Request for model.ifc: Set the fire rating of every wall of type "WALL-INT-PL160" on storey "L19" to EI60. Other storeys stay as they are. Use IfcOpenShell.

First a look at what the model holds.

```python
import ifcopenshell
import ifcopenshell.util.element

model = ifcopenshell.open("model.ifc")
print(model.schema)
storey = next(s for s in model.by_type("IfcBuildingStorey") if s.Name == "L19")
walls = [e for e in ifcopenshell.util.element.get_decomposition(storey) if e.is_a("IfcWall")]
seen = {}
for e in walls:
    element_type = ifcopenshell.util.element.get_type(e)
    key = (element_type.Name if element_type != e and element_type else None, ifcopenshell.util.element.get_pset(e, "Pset_WallCommon", "FireRating"))
    seen[key] = seen.get(key, 0) + 1
for (name, value), count in sorted(seen.items(), key=str):
    print(count, "x", name, "|", value)
```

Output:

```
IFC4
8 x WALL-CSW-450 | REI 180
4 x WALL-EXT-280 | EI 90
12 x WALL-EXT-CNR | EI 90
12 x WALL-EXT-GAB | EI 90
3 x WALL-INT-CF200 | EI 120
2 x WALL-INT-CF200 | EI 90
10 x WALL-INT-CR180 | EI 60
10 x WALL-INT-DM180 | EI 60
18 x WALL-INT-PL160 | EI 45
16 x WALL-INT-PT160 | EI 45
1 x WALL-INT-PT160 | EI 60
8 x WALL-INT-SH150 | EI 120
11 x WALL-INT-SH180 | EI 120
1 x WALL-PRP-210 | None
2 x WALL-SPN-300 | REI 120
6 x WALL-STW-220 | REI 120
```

```python
import ifcopenshell
import ifcopenshell.api.pset
import ifcopenshell.util.element

model = ifcopenshell.open("model.ifc")

storey = next(s for s in model.by_type("IfcBuildingStorey") if s.Name == "L19")
walls = [e for e in ifcopenshell.util.element.get_decomposition(storey) if e.is_a("IfcWall")]

count = 0
for e in walls:
    element_type = ifcopenshell.util.element.get_type(e)
    if element_type in (None, e) or element_type.Name != "WALL-INT-PL160":
        continue
    # add_pset returns the element's existing set when there is one.
    pset = ifcopenshell.api.pset.add_pset(model, product=e, name="Pset_WallCommon")
    ifcopenshell.api.pset.edit_pset(model, pset=pset, properties={"FireRating": "EI60"})
    count += 1

print(count, "walls updated")

model.write("model_rev.ifc")
```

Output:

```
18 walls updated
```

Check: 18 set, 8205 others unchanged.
